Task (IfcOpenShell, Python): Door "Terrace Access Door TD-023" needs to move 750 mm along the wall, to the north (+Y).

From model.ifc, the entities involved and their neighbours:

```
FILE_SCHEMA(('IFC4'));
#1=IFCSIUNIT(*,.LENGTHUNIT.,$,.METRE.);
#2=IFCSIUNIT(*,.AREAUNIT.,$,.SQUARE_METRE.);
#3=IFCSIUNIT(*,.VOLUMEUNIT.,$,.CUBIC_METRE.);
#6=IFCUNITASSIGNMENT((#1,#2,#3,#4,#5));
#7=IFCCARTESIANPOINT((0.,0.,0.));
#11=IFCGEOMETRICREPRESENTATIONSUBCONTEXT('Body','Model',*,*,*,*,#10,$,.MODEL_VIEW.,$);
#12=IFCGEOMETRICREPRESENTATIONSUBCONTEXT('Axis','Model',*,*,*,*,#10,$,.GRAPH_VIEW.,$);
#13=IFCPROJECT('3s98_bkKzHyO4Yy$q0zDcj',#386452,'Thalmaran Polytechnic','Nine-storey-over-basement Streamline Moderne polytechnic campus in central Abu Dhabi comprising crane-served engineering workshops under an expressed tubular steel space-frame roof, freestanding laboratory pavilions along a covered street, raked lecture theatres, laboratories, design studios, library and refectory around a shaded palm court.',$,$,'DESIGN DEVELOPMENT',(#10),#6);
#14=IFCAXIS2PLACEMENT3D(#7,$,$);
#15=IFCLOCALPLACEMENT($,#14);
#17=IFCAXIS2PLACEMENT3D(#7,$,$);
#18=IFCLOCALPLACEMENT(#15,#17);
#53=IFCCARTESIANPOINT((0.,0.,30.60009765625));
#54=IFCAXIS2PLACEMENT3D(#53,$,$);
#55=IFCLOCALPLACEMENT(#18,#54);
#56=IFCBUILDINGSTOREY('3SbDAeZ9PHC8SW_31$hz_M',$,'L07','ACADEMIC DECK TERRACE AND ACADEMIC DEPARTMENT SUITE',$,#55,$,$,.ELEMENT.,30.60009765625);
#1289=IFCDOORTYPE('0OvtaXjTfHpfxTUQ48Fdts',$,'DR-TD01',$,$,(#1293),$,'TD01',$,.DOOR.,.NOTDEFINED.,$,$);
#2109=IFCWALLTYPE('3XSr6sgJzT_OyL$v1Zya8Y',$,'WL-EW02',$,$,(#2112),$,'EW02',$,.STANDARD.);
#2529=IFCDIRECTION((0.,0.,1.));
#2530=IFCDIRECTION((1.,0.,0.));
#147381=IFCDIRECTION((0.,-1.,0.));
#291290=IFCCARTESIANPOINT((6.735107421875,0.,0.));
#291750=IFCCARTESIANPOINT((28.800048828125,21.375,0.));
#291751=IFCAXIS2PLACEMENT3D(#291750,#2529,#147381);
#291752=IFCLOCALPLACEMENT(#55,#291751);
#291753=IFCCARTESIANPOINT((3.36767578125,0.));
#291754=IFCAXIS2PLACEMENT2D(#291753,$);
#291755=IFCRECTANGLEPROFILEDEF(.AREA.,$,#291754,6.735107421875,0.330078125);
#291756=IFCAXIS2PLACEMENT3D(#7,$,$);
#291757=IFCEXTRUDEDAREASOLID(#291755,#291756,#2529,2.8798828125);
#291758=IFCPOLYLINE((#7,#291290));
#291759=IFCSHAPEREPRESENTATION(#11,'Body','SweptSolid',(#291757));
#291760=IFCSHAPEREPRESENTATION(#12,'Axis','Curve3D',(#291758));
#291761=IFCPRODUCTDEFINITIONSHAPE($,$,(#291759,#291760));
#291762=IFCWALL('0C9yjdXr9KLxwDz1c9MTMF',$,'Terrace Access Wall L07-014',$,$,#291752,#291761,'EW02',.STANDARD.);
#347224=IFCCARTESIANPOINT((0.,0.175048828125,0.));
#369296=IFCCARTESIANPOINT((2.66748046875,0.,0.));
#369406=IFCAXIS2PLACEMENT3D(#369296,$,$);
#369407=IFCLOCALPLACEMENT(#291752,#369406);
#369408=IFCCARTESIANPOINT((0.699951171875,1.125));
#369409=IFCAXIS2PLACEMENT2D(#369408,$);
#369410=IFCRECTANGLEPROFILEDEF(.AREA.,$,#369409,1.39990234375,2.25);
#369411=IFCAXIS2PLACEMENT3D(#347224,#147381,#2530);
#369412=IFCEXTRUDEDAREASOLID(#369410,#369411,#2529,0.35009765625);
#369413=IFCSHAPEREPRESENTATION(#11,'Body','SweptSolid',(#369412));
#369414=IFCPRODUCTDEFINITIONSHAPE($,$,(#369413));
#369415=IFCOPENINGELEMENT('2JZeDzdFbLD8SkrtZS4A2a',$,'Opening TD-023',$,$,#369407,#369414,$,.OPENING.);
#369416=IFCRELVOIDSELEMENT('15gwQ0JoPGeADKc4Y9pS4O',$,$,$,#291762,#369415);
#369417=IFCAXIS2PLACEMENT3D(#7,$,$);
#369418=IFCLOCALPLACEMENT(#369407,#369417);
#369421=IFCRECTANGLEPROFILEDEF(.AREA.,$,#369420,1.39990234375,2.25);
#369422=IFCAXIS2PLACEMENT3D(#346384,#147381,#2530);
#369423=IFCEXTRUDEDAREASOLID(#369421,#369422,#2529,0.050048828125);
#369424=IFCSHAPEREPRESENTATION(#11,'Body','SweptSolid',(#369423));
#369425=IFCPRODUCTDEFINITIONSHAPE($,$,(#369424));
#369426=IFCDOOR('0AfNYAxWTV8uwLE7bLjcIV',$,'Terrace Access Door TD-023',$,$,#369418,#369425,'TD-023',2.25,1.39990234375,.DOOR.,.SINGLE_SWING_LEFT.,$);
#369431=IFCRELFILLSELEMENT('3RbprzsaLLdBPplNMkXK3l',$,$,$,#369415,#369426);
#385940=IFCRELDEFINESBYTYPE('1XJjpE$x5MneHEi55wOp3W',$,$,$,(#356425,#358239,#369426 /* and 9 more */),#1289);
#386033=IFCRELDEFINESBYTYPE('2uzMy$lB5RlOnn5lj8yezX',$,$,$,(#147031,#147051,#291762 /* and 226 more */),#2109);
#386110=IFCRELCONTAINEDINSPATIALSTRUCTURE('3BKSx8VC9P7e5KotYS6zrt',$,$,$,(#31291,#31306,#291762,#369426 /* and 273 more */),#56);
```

```python
import ifcopenshell
import ifcopenshell.api.geometry
import ifcopenshell.util.placement

model = ifcopenshell.open("model.ifc")

door = model.by_guid("0AfNYAxWTV8uwLE7bLjcIV")
opening = door.FillsVoids[0].RelatingOpeningElement
wall = opening.VoidsElements[0].RelatingBuildingElement

wall_matrix = ifcopenshell.util.placement.get_local_placement(wall.ObjectPlacement)
shift = wall_matrix[:3, 0] * -0.75
before = ifcopenshell.util.placement.get_local_placement(door.ObjectPlacement)[:3, 3].copy()

# The door is placed relative to its opening, so it follows when the opening moves.
matrix = ifcopenshell.util.placement.get_local_placement(opening.ObjectPlacement)
matrix[:3, 3] += shift
ifcopenshell.api.geometry.edit_object_placement(
    model, product=opening, matrix=matrix, is_si=False, should_transform_children=True
)

after = ifcopenshell.util.placement.get_local_placement(door.ObjectPlacement)[:3, 3]
print("door moved by", (after - before).round(3) + 0.0)

model.write("model_v2.ifc")
```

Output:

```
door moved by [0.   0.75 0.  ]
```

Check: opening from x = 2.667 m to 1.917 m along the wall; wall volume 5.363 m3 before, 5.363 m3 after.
